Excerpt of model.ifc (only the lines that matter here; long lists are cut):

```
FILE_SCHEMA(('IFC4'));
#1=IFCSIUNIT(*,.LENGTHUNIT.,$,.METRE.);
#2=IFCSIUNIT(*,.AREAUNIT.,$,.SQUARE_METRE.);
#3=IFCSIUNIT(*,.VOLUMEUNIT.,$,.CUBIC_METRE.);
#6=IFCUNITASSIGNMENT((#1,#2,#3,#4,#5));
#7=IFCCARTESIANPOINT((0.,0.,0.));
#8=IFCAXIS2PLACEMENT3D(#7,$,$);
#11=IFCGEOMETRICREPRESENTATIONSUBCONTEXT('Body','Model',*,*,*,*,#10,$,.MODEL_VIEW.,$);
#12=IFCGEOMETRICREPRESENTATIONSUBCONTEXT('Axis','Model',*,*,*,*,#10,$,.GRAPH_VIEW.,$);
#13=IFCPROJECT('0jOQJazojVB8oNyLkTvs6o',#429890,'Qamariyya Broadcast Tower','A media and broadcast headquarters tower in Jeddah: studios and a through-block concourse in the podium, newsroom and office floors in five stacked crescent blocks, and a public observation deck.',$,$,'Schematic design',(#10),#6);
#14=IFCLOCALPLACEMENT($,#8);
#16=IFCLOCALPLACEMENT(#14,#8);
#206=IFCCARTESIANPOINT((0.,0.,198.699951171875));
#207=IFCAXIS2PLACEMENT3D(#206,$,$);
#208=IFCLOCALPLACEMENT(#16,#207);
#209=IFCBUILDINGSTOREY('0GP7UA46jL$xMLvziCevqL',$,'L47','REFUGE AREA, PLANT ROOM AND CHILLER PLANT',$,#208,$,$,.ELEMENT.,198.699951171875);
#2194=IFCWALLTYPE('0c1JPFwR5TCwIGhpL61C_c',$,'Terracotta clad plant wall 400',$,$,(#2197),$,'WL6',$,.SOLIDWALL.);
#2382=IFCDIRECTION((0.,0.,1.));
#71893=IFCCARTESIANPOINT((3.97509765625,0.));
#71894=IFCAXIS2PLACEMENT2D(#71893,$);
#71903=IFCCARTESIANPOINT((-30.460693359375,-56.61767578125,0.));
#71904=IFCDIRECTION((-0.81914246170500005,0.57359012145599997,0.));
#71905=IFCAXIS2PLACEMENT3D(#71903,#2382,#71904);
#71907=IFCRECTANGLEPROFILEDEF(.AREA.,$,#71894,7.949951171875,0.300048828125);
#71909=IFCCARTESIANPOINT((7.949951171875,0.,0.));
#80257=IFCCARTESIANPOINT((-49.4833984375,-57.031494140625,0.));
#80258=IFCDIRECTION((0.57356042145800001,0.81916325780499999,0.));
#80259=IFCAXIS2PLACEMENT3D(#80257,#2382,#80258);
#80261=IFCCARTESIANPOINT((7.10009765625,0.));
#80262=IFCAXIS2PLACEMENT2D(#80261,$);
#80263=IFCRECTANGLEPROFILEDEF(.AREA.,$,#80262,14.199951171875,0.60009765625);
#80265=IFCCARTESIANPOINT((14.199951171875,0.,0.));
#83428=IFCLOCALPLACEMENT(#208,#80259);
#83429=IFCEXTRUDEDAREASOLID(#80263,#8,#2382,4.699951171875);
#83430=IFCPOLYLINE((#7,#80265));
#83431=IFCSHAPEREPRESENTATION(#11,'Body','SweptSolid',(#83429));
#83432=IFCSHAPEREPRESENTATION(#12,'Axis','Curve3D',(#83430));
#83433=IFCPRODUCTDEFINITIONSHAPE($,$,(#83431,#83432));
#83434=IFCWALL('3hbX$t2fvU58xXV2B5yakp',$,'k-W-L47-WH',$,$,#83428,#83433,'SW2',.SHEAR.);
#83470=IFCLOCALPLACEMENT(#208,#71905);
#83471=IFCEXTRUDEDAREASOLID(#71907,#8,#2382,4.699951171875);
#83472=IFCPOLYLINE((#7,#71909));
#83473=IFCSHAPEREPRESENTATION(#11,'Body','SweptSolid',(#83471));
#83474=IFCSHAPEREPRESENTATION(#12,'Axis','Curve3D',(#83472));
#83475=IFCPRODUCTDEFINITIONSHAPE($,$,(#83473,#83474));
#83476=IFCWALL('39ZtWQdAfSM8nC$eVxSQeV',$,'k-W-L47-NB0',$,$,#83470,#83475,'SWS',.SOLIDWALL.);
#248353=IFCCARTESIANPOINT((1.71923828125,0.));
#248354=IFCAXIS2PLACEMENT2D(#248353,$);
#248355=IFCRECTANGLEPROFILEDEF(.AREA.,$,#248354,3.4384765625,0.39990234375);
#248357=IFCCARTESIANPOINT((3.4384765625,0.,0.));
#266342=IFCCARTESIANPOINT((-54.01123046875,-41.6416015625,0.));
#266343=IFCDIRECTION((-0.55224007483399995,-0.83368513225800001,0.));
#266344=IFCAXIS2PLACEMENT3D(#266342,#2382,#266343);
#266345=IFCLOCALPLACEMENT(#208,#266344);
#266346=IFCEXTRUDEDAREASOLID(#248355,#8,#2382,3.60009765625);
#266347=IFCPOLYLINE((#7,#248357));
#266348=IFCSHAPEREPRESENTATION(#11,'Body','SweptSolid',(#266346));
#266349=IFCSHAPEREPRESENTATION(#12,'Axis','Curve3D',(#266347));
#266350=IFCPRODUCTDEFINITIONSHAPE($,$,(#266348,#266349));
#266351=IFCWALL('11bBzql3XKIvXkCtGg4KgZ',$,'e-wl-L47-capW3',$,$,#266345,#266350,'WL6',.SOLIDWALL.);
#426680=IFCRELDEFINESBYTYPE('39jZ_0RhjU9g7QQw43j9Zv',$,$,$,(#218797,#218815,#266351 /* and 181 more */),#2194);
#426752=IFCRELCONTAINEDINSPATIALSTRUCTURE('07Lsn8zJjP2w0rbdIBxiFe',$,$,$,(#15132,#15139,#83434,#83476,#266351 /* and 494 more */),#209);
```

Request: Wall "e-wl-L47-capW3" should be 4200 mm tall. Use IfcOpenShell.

```python
import ifcopenshell
import ifcopenshell.geom
import ifcopenshell.util.representation
import ifcopenshell.util.shape
import ifcopenshell.util.unit

model = ifcopenshell.open("model.ifc")
unit_scale = ifcopenshell.util.unit.calculate_unit_scale(model)
settings = ifcopenshell.geom.settings()


def volume(element):
    """Net volume in cubic metres, openings subtracted."""
    shape = ifcopenshell.geom.create_shape(settings, element)
    return ifcopenshell.util.shape.get_volume(shape.geometry)


wall = model.by_id(266351)
before = volume(wall)

body = ifcopenshell.util.representation.get_representation(wall, "Model", "Body")
solid = body.Items[0]
old_height = solid.Depth
solid.Depth = 4.2 / unit_scale
after = volume(wall)

print(f"height {old_height:g} -> {solid.Depth:g}, volume {before:.3f} -> {after:.3f} m3")

model.write("model_edited.ifc")
```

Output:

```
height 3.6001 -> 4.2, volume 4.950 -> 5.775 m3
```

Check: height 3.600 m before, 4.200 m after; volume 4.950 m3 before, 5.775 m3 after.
